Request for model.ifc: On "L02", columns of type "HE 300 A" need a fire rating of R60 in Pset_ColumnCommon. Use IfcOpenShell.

First a look at what the model holds.

```python
import ifcopenshell
import ifcopenshell.util.element

model = ifcopenshell.open("model.ifc")
print(model.schema)
storey = next(s for s in model.by_type("IfcBuildingStorey") if s.Name == "L02")
columns = [e for e in ifcopenshell.util.element.get_decomposition(storey) if e.is_a("IfcColumn")]
seen = {}
for e in columns:
    element_type = ifcopenshell.util.element.get_type(e)
    key = (element_type.Name if element_type != e and element_type else None, ifcopenshell.util.element.get_pset(e, "Pset_ColumnCommon", "FireRating"))
    seen[key] = seen.get(key, 0) + 1
for (name, value), count in sorted(seen.items(), key=str):
    print(count, "x", name, "|", value)
```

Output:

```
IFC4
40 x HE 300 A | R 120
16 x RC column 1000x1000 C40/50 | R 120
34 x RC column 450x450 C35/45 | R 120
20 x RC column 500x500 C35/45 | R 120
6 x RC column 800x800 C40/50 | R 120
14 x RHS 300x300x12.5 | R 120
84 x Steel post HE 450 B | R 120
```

```python
import ifcopenshell
import ifcopenshell.api.pset
import ifcopenshell.util.element

model = ifcopenshell.open("model.ifc")

storey = next(s for s in model.by_type("IfcBuildingStorey") if s.Name == "L02")
columns = [e for e in ifcopenshell.util.element.get_decomposition(storey) if e.is_a("IfcColumn")]

count = 0
for e in columns:
    element_type = ifcopenshell.util.element.get_type(e)
    if element_type in (None, e) or element_type.Name != "HE 300 A":
        continue
    # add_pset returns the element's existing set when there is one.
    pset = ifcopenshell.api.pset.add_pset(model, product=e, name="Pset_ColumnCommon")
    ifcopenshell.api.pset.edit_pset(model, pset=pset, properties={"FireRating": "R60"})
    count += 1

print(count, "columns updated")

model.write("model_rev.ifc")
```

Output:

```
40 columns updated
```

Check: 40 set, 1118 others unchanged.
